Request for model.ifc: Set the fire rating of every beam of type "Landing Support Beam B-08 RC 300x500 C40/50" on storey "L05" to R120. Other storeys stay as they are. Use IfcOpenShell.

First a look at what the model holds.

```python
import ifcopenshell
import ifcopenshell.util.element

model = ifcopenshell.open("model.ifc")
print(model.schema)
storey = next(s for s in model.by_type("IfcBuildingStorey") if s.Name == "L05")
beams = [e for e in ifcopenshell.util.element.get_decomposition(storey) if e.is_a("IfcBeam")]
seen = {}
for e in beams:
    element_type = ifcopenshell.util.element.get_type(e)
    key = (element_type.Name if element_type != e and element_type else None, ifcopenshell.util.element.get_pset(e, "Pset_BeamCommon", "FireRating"))
    seen[key] = seen.get(key, 0) + 1
for (name, value), count in sorted(seen.items(), key=str):
    print(count, "x", name, "|", value)
```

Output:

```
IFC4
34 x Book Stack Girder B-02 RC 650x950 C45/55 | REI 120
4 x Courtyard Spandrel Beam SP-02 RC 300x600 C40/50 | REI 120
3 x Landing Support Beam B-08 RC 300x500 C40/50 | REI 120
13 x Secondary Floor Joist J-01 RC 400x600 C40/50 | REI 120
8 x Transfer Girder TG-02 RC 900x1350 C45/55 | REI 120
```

```python
import ifcopenshell
import ifcopenshell.api.pset
import ifcopenshell.util.element

model = ifcopenshell.open("model.ifc")

storey = next(s for s in model.by_type("IfcBuildingStorey") if s.Name == "L05")
beams = [e for e in ifcopenshell.util.element.get_decomposition(storey) if e.is_a("IfcBeam")]

count = 0
for e in beams:
    element_type = ifcopenshell.util.element.get_type(e)
    if element_type in (None, e) or element_type.Name != "Landing Support Beam B-08 RC 300x500 C40/50":
        continue
    # add_pset returns the element's existing set when there is one.
    pset = ifcopenshell.api.pset.add_pset(model, product=e, name="Pset_BeamCommon")
    ifcopenshell.api.pset.edit_pset(model, pset=pset, properties={"FireRating": "R120"})
    count += 1

print(count, "beams updated")

model.write("model_edited.ifc")
```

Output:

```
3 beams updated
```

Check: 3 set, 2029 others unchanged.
